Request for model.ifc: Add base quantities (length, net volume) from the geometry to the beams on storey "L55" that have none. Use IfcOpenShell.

First a look at what the model holds.

```python
import ifcopenshell
import ifcopenshell.util.element
import ifcopenshell.util.unit

model = ifcopenshell.open("model.ifc")
print(model.schema)
for unit_type in ("LENGTHUNIT", "AREAUNIT", "VOLUMEUNIT"):
    print(unit_type, ifcopenshell.util.unit.calculate_unit_scale(model, unit_type))
storey = next(s for s in model.by_type("IfcBuildingStorey") if s.Name == "L55")
beams = [e for e in ifcopenshell.util.element.get_decomposition(storey) if e.is_a("IfcBeam")]
for e in sorted(beams, key=lambda e: e.id()):
    print(e.id(), e.is_a(), e.Name, list(ifcopenshell.util.element.get_psets(e, qtos_only=True)), sep=" | ")
```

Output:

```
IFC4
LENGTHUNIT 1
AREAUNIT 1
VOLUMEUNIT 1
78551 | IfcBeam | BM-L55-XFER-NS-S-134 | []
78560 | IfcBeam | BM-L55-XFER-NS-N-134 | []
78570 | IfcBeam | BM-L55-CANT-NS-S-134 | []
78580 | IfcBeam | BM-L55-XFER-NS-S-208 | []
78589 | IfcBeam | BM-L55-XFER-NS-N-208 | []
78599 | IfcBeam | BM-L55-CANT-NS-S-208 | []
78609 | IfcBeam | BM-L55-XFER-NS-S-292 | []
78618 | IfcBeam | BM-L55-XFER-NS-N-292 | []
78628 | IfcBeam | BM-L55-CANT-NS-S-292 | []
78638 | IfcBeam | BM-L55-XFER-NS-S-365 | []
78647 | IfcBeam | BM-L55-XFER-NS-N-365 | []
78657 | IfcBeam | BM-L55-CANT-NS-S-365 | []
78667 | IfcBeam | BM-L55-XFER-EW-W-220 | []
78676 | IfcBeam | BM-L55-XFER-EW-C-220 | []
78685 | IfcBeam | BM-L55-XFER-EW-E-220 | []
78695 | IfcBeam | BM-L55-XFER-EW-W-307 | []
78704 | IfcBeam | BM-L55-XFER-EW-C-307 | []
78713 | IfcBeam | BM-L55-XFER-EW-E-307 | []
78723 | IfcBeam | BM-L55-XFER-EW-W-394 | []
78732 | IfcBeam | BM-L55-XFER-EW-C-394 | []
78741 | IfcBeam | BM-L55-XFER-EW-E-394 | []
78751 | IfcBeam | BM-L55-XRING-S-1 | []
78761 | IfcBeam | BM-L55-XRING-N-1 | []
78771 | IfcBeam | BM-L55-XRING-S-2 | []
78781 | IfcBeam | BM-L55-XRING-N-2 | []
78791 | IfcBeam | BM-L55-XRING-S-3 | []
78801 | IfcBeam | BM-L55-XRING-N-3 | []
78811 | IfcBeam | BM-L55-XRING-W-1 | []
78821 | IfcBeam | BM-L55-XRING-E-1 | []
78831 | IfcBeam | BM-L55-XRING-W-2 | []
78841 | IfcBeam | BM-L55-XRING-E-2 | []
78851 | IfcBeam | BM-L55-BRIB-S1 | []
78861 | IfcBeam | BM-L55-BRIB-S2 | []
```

```python
import ifcopenshell
import ifcopenshell.api.pset
import ifcopenshell.geom
import ifcopenshell.util.element
import ifcopenshell.util.shape
import ifcopenshell.util.unit

model = ifcopenshell.open("model.ifc")
unit_scale = ifcopenshell.util.unit.calculate_unit_scale(model)
volume_scale = ifcopenshell.util.unit.calculate_unit_scale(model, "VOLUMEUNIT")
settings = ifcopenshell.geom.settings()

storey = next(s for s in model.by_type("IfcBuildingStorey") if s.Name == "L55")
beams = [e for e in ifcopenshell.util.element.get_decomposition(storey) if e.is_a("IfcBeam")]

for e in sorted(beams, key=lambda e: e.id()):
    if ifcopenshell.util.element.get_psets(e, qtos_only=True, should_inherit=False):
        continue
    # Geometry comes back in metres, in the element's own axes.
    shape = ifcopenshell.geom.create_shape(settings, e)
    values = {
        "Length": ifcopenshell.util.shape.get_max_xyz(shape.geometry) / unit_scale,
        "NetVolume": ifcopenshell.util.shape.get_volume(shape.geometry) / volume_scale,
    }
    qto = ifcopenshell.api.pset.add_qto(model, product=e, name="Qto_BeamBaseQuantities")
    ifcopenshell.api.pset.edit_qto(model, qto=qto, properties=values)
    print(e.id(), {k: round(v, 3) for k, v in values.items()})

model.write("model_updated.ifc")
```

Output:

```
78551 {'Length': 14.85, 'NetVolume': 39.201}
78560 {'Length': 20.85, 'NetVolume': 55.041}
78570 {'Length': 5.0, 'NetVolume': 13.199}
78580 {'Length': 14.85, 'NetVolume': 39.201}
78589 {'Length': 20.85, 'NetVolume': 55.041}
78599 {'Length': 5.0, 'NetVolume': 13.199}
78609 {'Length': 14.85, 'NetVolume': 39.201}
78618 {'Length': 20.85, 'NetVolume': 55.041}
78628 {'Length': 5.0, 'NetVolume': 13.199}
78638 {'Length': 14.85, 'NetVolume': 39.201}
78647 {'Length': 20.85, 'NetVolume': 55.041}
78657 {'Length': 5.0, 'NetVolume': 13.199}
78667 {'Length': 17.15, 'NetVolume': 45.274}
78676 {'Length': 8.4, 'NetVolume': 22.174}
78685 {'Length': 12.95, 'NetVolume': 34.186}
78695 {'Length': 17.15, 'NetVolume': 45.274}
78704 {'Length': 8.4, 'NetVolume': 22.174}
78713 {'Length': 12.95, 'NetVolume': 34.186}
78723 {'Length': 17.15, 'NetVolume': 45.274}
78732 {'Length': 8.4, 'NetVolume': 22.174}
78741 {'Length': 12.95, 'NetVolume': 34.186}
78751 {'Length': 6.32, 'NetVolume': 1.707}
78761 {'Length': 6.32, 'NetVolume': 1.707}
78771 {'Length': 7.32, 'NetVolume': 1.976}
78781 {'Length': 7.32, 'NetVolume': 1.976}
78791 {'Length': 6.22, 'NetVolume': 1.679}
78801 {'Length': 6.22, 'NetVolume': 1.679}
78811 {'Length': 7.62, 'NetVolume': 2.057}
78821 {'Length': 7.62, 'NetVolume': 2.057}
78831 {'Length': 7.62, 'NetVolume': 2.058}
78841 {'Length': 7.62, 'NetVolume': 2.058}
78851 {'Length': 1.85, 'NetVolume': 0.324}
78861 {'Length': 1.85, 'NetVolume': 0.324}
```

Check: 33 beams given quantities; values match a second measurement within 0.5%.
